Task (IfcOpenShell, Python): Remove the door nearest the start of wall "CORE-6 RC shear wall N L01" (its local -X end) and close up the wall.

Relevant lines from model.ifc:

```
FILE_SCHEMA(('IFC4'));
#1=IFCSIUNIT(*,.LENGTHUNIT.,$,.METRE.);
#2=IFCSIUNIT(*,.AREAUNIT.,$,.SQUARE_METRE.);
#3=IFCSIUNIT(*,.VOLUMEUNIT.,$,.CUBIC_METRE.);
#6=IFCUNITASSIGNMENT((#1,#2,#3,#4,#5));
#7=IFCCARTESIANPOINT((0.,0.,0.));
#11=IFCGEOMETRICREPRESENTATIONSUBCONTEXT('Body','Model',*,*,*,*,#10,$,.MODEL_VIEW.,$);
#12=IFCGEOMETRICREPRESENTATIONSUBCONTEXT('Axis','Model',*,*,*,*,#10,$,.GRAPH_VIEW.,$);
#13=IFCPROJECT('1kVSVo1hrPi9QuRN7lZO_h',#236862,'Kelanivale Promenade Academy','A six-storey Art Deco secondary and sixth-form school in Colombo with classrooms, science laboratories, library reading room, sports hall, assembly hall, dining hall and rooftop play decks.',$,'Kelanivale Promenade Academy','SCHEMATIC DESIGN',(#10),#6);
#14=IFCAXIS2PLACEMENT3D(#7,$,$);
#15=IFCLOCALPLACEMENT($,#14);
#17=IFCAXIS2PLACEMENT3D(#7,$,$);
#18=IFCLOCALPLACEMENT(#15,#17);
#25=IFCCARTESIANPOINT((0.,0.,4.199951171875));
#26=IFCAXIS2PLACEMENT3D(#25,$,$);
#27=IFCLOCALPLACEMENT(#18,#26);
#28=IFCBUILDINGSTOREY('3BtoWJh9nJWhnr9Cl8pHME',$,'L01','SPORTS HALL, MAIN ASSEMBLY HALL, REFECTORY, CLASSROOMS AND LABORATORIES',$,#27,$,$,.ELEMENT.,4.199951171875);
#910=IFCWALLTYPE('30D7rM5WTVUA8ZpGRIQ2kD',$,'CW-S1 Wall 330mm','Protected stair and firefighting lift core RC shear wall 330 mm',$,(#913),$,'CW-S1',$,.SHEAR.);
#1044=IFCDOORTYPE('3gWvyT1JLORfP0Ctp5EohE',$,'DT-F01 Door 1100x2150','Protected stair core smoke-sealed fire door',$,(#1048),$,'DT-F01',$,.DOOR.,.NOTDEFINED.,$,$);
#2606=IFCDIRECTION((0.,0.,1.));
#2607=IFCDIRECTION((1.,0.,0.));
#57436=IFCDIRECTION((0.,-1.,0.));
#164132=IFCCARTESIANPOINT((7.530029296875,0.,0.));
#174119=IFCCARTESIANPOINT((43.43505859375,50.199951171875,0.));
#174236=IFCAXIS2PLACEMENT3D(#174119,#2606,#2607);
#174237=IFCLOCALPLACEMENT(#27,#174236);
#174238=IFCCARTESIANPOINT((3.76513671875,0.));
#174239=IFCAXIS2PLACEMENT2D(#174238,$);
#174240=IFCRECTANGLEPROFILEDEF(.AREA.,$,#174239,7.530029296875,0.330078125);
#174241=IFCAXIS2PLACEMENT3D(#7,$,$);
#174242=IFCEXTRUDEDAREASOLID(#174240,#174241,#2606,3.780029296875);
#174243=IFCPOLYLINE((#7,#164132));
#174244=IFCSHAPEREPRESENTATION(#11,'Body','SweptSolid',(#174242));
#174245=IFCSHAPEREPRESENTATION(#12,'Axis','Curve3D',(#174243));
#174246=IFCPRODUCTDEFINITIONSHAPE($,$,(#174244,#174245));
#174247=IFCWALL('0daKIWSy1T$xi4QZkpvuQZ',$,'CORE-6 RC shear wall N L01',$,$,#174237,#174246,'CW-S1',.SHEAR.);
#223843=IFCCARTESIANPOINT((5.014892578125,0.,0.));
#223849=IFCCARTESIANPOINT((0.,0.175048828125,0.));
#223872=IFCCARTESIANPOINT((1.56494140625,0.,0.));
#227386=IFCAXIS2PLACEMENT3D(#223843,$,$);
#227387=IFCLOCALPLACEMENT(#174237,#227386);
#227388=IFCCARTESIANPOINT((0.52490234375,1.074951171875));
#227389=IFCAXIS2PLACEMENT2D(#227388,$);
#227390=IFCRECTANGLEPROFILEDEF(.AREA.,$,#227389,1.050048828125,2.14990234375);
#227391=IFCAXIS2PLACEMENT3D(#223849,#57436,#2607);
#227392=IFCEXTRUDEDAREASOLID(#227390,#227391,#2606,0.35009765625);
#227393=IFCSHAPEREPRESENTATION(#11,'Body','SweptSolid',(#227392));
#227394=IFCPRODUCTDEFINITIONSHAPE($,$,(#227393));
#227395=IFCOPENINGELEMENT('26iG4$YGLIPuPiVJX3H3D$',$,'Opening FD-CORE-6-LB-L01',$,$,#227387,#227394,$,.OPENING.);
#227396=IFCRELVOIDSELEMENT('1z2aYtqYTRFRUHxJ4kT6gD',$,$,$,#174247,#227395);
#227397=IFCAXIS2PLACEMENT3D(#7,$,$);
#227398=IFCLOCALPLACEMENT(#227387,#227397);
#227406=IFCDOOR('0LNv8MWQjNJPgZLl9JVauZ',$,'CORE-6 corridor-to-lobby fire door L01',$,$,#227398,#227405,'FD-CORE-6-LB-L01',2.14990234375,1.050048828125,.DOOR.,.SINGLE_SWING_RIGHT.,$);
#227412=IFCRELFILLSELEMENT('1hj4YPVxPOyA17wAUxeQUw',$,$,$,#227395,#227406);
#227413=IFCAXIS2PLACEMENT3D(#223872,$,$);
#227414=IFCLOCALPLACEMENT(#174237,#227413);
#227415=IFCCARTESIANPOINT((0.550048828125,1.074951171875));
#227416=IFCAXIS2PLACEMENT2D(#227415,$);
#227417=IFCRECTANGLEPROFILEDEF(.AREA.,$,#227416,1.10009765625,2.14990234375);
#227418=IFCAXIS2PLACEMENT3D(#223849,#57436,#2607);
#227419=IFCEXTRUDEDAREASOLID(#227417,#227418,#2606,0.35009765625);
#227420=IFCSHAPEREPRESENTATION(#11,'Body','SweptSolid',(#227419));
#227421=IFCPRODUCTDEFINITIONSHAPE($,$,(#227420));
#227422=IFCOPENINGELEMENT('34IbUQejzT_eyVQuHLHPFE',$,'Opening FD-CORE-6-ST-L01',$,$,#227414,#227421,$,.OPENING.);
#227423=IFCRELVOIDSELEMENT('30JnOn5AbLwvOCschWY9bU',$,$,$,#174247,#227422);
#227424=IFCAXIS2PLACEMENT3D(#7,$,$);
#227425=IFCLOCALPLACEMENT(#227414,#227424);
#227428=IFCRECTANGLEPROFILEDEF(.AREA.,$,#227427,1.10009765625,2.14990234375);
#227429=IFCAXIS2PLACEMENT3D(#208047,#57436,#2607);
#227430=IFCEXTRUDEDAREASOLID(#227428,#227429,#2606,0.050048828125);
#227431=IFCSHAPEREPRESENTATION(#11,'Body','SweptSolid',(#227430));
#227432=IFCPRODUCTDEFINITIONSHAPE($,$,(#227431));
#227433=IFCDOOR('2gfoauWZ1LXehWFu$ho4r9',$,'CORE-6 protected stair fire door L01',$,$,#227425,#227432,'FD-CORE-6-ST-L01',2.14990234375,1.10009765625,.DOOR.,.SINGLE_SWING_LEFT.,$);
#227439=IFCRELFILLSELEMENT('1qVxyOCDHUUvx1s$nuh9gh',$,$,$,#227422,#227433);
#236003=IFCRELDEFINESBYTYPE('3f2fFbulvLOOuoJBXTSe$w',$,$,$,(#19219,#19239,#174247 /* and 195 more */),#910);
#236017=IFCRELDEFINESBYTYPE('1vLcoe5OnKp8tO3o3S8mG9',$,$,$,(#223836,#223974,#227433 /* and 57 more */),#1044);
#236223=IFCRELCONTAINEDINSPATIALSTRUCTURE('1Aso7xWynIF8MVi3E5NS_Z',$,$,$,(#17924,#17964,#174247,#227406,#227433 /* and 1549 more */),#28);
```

```python
import ifcopenshell
import ifcopenshell.api.feature
import ifcopenshell.api.root
import ifcopenshell.geom
import ifcopenshell.util.shape

model = ifcopenshell.open("model.ifc")
settings = ifcopenshell.geom.settings()


def volume(element):
    """Net volume in cubic metres, openings subtracted."""
    shape = ifcopenshell.geom.create_shape(settings, element)
    return ifcopenshell.util.shape.get_volume(shape.geometry)


door = model.by_guid("2gfoauWZ1LXehWFu$ho4r9")
opening = door.FillsVoids[0].RelatingOpeningElement
wall = opening.VoidsElements[0].RelatingBuildingElement
before = volume(wall)

ifcopenshell.api.root.remove_product(model, product=door)
ifcopenshell.api.feature.remove_feature(model, feature=opening)

after = volume(wall)

print(f"wall volume {before:.3f} -> {after:.3f} m3")

model.write("model_updated.ifc")
```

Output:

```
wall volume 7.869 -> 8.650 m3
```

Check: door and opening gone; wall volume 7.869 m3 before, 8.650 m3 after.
